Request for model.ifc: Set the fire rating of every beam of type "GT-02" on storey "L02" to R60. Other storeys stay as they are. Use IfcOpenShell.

First a look at what the model holds.

```python
import ifcopenshell
import ifcopenshell.util.element

model = ifcopenshell.open("model.ifc")
print(model.schema)
storey = next(s for s in model.by_type("IfcBuildingStorey") if s.Name == "L02")
beams = [e for e in ifcopenshell.util.element.get_decomposition(storey) if e.is_a("IfcBeam")]
seen = {}
for e in beams:
    element_type = ifcopenshell.util.element.get_type(e)
    key = (element_type.Name if element_type != e and element_type else None, ifcopenshell.util.element.get_pset(e, "Pset_BeamCommon", "FireRating"))
    seen[key] = seen.get(key, 0) + 1
for (name, value), count in sorted(seen.items(), key=str):
    print(count, "x", name, "|", value)
```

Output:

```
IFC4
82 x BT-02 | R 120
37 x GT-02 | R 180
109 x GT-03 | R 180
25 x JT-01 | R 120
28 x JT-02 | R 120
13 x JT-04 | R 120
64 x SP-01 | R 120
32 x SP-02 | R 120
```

```python
import ifcopenshell
import ifcopenshell.api.pset
import ifcopenshell.util.element

model = ifcopenshell.open("model.ifc")

storey = next(s for s in model.by_type("IfcBuildingStorey") if s.Name == "L02")
beams = [e for e in ifcopenshell.util.element.get_decomposition(storey) if e.is_a("IfcBeam")]

count = 0
for e in beams:
    element_type = ifcopenshell.util.element.get_type(e)
    if element_type in (None, e) or element_type.Name != "GT-02":
        continue
    # add_pset returns the element's existing set when there is one.
    pset = ifcopenshell.api.pset.add_pset(model, product=e, name="Pset_BeamCommon")
    ifcopenshell.api.pset.edit_pset(model, pset=pset, properties={"FireRating": "R60"})
    count += 1

print(count, "beams updated")

model.write("model_updated.ifc")
```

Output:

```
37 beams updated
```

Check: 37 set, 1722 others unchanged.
